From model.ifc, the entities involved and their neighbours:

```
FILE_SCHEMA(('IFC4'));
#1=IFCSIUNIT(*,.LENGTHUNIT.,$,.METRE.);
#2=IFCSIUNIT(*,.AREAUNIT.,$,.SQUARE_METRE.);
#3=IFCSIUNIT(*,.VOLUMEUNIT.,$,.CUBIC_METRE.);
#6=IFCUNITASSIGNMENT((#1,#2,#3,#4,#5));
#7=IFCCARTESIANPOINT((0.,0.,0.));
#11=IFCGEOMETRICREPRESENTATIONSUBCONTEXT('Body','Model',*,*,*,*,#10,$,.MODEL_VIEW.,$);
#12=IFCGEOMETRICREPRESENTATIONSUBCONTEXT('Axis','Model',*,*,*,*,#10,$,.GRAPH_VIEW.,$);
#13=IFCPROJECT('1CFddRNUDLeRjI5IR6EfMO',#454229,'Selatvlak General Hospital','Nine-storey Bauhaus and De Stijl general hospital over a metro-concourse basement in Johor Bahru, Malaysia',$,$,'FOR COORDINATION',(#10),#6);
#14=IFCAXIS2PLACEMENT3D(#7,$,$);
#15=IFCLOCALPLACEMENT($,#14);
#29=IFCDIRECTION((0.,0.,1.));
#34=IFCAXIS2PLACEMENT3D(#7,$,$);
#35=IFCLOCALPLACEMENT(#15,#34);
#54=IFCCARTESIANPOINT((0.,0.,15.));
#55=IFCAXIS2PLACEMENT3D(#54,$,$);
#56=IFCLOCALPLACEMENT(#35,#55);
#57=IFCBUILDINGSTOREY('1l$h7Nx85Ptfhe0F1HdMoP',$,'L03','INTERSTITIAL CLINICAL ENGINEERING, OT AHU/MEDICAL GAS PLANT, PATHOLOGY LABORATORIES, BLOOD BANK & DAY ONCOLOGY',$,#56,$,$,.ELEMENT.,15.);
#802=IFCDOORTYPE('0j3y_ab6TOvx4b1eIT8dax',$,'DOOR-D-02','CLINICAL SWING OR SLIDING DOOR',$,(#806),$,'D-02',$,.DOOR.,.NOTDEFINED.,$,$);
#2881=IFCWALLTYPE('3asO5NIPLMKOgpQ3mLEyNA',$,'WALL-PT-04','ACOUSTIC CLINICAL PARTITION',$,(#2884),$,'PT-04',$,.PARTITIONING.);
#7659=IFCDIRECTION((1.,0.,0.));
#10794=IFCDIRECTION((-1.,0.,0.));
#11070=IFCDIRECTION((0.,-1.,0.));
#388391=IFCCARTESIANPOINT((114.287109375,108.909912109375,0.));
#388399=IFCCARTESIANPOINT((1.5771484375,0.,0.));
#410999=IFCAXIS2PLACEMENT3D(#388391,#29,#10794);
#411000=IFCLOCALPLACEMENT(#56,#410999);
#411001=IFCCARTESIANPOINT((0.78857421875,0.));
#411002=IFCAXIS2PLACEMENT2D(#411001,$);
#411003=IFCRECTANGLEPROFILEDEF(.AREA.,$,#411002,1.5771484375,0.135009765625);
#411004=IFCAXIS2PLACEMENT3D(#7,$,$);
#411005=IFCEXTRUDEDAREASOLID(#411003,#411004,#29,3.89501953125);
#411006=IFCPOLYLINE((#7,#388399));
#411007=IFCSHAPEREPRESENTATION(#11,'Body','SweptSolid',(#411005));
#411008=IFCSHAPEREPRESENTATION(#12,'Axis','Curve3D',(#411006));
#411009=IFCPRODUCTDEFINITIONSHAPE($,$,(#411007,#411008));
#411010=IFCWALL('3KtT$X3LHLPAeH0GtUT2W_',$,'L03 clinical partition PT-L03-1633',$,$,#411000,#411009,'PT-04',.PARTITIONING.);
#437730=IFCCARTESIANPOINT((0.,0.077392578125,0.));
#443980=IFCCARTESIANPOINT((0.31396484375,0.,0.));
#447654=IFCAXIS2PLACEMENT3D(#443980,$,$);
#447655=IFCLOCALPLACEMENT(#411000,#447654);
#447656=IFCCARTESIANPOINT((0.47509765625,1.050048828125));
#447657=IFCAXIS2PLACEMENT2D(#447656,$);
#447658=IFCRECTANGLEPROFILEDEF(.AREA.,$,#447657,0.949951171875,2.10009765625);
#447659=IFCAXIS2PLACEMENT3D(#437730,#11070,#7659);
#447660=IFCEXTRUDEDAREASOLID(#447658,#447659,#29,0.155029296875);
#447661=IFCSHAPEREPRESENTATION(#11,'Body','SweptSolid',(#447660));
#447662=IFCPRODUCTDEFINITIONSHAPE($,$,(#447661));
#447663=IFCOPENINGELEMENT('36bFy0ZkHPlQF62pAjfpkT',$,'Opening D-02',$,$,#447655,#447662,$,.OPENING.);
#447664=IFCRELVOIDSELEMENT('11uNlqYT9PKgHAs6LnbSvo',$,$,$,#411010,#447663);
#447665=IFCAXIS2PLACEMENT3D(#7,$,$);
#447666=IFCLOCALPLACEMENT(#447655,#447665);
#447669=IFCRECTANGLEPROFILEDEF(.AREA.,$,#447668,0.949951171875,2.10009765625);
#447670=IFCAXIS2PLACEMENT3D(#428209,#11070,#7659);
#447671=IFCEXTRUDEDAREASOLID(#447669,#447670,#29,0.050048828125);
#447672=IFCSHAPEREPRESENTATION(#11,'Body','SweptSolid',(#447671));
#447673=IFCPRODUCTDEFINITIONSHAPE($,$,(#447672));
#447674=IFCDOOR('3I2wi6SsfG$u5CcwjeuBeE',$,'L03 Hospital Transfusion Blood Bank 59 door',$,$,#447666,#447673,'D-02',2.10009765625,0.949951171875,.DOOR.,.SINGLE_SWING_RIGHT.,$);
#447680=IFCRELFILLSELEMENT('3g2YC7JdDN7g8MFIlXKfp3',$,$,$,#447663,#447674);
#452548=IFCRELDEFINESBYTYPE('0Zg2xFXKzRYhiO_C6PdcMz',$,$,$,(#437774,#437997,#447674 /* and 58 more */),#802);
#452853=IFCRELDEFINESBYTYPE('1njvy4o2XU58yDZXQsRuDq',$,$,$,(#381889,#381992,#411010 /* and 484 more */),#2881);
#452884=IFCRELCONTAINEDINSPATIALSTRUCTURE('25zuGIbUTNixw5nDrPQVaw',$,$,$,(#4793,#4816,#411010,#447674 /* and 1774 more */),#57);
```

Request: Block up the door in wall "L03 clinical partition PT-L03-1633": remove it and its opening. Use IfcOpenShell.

```python
import ifcopenshell
import ifcopenshell.api.feature
import ifcopenshell.api.root
import ifcopenshell.geom
import ifcopenshell.util.shape

model = ifcopenshell.open("model.ifc")
settings = ifcopenshell.geom.settings()


def volume(element):
    """Net volume in cubic metres, openings subtracted."""
    shape = ifcopenshell.geom.create_shape(settings, element)
    return ifcopenshell.util.shape.get_volume(shape.geometry)


door = model.by_guid("3I2wi6SsfG$u5CcwjeuBeE")
opening = door.FillsVoids[0].RelatingOpeningElement
wall = opening.VoidsElements[0].RelatingBuildingElement
before = volume(wall)

ifcopenshell.api.root.remove_product(model, product=door)
ifcopenshell.api.feature.remove_feature(model, feature=opening)

after = volume(wall)

print(f"wall volume {before:.3f} -> {after:.3f} m3")

model.write("model-out.ifc")
```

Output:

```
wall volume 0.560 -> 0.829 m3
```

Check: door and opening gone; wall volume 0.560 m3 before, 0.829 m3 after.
